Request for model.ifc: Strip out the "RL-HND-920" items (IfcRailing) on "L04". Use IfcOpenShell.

First a look at what the model holds.

```python
import ifcopenshell
import ifcopenshell.util.element

model = ifcopenshell.open("model.ifc")
print(model.schema)
storey = next(s for s in model.by_type("IfcBuildingStorey") if s.Name == "L04")
railings = [e for e in ifcopenshell.util.element.get_decomposition(storey) if e.is_a("IfcRailing")]
seen = {}
for e in railings:
    element_type = ifcopenshell.util.element.get_type(e)
    name = element_type.Name if element_type not in (None, e) else None
    seen[name] = seen.get(name, 0) + 1
for name, count in sorted(seen.items(), key=str):
    print(count, "x", name)
```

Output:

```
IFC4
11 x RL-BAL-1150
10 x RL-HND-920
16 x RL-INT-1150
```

```python
import ifcopenshell
import ifcopenshell.api.root
import ifcopenshell.util.element

model = ifcopenshell.open("model.ifc")

storey = next(s for s in model.by_type("IfcBuildingStorey") if s.Name == "L04")
railings = [e for e in ifcopenshell.util.element.get_decomposition(storey) if e.is_a("IfcRailing")]
targets = [e for e in railings if (t := ifcopenshell.util.element.get_type(e)) not in (None, e) and t.Name == "RL-HND-920"]

for e in targets:
    ifcopenshell.api.root.remove_product(model, product=e)
print(len(targets), "removed")

model.write("model_rev.ifc")
```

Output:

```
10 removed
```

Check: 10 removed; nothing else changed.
